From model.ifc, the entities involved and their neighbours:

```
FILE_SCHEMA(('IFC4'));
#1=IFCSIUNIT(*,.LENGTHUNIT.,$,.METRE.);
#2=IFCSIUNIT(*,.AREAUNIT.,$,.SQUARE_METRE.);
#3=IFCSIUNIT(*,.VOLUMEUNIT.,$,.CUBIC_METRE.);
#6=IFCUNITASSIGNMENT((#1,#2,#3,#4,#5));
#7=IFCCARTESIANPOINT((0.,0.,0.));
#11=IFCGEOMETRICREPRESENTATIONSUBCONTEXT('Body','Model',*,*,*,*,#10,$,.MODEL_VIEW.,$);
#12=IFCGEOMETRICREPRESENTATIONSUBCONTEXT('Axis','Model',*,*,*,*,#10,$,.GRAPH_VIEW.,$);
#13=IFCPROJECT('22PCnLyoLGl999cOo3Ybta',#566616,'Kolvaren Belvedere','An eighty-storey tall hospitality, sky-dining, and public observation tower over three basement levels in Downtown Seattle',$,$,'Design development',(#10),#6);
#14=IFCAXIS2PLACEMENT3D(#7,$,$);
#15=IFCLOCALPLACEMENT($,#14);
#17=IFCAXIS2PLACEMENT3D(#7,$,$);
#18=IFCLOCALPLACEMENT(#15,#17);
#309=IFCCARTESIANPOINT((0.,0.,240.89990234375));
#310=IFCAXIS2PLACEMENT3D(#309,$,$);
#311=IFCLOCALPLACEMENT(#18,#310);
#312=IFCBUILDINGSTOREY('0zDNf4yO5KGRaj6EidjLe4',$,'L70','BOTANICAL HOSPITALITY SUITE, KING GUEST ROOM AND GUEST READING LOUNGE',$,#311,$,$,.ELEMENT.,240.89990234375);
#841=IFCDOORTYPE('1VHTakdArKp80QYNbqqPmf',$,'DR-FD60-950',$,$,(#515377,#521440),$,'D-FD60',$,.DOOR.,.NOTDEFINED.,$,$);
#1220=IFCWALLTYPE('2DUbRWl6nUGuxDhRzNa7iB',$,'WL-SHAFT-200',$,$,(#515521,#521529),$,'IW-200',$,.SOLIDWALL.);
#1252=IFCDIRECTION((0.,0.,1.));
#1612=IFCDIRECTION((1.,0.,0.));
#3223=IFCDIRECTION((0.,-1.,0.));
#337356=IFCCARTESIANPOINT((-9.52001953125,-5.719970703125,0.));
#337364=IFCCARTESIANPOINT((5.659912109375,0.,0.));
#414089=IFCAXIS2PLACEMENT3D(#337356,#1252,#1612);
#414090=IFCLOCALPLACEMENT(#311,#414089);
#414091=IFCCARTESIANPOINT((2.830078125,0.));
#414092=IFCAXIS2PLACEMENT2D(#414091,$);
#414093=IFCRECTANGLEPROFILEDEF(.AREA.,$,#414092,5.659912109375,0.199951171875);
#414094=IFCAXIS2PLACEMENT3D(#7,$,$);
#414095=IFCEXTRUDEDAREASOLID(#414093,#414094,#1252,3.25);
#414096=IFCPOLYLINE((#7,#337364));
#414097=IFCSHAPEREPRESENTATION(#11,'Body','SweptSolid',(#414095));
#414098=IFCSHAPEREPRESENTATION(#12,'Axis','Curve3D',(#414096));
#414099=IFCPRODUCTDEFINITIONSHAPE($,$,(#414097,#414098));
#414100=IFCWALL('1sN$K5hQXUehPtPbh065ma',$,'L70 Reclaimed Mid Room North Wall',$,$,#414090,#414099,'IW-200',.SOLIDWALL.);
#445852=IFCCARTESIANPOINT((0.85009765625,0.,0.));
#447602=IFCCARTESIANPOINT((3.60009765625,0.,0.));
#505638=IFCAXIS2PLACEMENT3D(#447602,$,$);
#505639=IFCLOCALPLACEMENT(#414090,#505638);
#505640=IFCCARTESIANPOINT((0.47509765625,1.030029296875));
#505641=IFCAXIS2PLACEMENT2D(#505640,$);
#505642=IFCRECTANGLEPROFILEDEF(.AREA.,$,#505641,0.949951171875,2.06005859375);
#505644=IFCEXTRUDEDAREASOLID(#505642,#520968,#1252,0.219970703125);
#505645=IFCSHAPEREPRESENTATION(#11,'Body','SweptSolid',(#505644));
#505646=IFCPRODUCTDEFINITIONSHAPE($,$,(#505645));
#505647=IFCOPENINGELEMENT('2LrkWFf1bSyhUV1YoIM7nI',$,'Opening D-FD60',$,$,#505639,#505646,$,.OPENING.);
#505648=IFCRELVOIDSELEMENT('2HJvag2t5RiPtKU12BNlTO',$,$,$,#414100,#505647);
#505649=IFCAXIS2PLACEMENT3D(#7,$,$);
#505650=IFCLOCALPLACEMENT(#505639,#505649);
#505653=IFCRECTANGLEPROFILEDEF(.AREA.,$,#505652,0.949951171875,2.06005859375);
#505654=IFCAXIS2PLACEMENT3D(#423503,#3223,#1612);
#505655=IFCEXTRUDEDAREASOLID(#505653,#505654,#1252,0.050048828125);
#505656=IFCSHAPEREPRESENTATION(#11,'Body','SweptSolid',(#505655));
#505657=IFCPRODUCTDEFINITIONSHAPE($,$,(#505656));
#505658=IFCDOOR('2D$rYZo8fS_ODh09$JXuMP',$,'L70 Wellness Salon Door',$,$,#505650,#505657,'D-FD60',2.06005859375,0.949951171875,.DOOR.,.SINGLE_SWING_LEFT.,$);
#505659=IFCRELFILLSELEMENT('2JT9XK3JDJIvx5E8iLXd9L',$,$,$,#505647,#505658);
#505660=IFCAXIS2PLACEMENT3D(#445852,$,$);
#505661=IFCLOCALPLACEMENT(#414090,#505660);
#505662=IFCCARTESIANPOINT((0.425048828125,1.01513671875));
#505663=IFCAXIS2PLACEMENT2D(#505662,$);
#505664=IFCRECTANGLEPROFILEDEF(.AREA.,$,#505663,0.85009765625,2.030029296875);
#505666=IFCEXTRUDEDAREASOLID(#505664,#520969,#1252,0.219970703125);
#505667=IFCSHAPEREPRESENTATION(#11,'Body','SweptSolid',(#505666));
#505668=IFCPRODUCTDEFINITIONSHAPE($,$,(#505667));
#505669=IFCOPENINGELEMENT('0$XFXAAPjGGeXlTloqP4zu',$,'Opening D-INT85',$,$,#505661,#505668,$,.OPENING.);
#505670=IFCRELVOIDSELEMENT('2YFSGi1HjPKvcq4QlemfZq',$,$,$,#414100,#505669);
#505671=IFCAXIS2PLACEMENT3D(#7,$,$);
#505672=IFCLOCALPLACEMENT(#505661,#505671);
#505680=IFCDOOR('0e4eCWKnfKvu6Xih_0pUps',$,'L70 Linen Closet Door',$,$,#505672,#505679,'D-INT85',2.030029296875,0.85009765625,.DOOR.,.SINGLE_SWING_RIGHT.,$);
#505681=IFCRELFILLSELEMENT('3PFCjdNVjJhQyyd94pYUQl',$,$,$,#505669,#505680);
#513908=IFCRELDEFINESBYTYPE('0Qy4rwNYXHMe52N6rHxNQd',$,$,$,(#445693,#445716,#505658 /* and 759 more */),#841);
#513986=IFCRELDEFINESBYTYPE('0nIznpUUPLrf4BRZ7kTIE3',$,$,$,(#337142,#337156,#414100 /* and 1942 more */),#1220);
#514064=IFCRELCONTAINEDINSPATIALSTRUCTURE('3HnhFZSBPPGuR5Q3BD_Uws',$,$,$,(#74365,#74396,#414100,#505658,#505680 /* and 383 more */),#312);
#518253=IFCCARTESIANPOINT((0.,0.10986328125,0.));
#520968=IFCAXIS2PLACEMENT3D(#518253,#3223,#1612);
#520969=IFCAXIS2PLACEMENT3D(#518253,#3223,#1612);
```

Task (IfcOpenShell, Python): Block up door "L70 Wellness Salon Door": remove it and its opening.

```python
import ifcopenshell
import ifcopenshell.api.feature
import ifcopenshell.api.root
import ifcopenshell.geom
import ifcopenshell.util.shape

model = ifcopenshell.open("model.ifc")
settings = ifcopenshell.geom.settings()


def volume(element):
    """Net volume in cubic metres, openings subtracted."""
    shape = ifcopenshell.geom.create_shape(settings, element)
    return ifcopenshell.util.shape.get_volume(shape.geometry)


door = model.by_id(505658)
opening = door.FillsVoids[0].RelatingOpeningElement
wall = opening.VoidsElements[0].RelatingBuildingElement
before = volume(wall)

ifcopenshell.api.root.remove_product(model, product=door)
ifcopenshell.api.feature.remove_feature(model, feature=opening)

after = volume(wall)

print(f"wall volume {before:.3f} -> {after:.3f} m3")

model.write("model_edited.ifc")
```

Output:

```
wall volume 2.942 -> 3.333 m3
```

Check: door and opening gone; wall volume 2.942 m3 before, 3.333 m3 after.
